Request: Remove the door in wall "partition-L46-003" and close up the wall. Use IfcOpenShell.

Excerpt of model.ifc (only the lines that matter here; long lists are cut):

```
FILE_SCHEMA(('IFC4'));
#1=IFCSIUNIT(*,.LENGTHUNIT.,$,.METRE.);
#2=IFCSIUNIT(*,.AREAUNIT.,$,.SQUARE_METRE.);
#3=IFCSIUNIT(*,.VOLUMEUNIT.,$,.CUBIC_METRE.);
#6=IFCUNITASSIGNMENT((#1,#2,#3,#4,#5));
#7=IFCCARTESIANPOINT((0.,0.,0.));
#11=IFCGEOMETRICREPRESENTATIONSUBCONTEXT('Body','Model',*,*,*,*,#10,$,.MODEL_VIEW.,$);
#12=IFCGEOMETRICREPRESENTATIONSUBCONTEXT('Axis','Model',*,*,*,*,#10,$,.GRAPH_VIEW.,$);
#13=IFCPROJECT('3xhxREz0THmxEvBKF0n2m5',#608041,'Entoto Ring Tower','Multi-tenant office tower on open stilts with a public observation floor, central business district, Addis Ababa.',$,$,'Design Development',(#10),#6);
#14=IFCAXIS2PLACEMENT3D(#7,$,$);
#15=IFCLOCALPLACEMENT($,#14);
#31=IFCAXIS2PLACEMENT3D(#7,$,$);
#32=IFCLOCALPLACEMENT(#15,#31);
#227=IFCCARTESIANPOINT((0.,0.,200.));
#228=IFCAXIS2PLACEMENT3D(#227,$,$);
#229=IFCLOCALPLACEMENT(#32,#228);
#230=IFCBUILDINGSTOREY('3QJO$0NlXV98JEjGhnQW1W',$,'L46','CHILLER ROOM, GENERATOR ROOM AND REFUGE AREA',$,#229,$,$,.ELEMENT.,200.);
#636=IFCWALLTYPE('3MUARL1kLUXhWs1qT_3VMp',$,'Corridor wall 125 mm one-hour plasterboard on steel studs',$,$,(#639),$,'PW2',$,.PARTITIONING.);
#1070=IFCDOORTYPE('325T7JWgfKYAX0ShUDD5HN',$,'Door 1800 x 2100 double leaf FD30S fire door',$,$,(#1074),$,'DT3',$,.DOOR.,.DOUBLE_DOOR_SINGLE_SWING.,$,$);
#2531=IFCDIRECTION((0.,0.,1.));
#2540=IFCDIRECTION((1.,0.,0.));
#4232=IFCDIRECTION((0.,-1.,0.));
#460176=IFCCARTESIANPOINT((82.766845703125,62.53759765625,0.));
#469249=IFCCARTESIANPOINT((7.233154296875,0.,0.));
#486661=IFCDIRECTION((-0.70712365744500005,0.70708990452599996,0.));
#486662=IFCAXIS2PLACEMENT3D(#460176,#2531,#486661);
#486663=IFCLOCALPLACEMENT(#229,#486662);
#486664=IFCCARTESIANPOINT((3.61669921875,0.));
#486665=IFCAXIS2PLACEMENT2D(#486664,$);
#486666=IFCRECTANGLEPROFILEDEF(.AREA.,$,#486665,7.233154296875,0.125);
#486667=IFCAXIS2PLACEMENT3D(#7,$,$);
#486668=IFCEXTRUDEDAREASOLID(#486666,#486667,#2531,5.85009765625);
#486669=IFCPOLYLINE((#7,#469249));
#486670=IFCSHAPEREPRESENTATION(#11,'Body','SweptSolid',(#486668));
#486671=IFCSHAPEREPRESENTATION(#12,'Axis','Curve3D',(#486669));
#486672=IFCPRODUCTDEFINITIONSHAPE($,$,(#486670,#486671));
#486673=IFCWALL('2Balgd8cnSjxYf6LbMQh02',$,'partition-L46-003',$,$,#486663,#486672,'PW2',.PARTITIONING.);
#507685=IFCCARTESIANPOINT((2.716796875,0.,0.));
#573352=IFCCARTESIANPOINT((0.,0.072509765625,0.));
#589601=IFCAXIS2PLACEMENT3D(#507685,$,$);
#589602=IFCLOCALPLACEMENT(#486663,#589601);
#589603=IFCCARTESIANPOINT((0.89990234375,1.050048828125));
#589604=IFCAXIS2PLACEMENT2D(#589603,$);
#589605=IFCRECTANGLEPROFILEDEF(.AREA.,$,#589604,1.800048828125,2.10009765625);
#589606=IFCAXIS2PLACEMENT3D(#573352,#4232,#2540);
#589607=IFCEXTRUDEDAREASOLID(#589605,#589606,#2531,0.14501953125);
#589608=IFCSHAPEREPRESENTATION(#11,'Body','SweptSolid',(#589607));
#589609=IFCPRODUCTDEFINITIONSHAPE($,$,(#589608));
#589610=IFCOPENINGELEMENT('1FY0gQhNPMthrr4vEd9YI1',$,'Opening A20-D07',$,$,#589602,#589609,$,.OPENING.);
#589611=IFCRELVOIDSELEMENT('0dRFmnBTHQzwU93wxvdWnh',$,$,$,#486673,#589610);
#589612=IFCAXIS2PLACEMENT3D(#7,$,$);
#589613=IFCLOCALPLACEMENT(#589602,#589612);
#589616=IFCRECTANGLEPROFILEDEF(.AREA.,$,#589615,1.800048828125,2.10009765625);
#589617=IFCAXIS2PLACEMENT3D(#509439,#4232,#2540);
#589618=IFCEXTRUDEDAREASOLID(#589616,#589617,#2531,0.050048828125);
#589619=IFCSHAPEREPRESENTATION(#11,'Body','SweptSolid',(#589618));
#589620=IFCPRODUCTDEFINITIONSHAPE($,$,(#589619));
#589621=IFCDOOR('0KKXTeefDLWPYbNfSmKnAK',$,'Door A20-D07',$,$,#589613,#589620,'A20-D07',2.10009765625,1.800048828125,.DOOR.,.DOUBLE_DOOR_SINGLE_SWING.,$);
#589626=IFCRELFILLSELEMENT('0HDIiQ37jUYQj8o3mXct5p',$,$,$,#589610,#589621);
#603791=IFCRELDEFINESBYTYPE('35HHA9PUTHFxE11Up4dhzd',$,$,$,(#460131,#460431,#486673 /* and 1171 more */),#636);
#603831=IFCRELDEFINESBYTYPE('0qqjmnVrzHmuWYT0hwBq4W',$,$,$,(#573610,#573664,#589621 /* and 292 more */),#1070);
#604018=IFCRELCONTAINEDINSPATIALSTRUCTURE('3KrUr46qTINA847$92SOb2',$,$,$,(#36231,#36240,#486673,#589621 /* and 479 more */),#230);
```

```python
import ifcopenshell
import ifcopenshell.api.feature
import ifcopenshell.api.root
import ifcopenshell.geom
import ifcopenshell.util.shape

model = ifcopenshell.open("model.ifc")
settings = ifcopenshell.geom.settings()


def volume(element):
    """Net volume in cubic metres, openings subtracted."""
    shape = ifcopenshell.geom.create_shape(settings, element)
    return ifcopenshell.util.shape.get_volume(shape.geometry)


door = model.by_id(589621)
opening = door.FillsVoids[0].RelatingOpeningElement
wall = opening.VoidsElements[0].RelatingBuildingElement
before = volume(wall)

ifcopenshell.api.root.remove_product(model, product=door)
ifcopenshell.api.feature.remove_feature(model, feature=opening)

after = volume(wall)

print(f"wall volume {before:.3f} -> {after:.3f} m3")

model.write("model_v2.ifc")
```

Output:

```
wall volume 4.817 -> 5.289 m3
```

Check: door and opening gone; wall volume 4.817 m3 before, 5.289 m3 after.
